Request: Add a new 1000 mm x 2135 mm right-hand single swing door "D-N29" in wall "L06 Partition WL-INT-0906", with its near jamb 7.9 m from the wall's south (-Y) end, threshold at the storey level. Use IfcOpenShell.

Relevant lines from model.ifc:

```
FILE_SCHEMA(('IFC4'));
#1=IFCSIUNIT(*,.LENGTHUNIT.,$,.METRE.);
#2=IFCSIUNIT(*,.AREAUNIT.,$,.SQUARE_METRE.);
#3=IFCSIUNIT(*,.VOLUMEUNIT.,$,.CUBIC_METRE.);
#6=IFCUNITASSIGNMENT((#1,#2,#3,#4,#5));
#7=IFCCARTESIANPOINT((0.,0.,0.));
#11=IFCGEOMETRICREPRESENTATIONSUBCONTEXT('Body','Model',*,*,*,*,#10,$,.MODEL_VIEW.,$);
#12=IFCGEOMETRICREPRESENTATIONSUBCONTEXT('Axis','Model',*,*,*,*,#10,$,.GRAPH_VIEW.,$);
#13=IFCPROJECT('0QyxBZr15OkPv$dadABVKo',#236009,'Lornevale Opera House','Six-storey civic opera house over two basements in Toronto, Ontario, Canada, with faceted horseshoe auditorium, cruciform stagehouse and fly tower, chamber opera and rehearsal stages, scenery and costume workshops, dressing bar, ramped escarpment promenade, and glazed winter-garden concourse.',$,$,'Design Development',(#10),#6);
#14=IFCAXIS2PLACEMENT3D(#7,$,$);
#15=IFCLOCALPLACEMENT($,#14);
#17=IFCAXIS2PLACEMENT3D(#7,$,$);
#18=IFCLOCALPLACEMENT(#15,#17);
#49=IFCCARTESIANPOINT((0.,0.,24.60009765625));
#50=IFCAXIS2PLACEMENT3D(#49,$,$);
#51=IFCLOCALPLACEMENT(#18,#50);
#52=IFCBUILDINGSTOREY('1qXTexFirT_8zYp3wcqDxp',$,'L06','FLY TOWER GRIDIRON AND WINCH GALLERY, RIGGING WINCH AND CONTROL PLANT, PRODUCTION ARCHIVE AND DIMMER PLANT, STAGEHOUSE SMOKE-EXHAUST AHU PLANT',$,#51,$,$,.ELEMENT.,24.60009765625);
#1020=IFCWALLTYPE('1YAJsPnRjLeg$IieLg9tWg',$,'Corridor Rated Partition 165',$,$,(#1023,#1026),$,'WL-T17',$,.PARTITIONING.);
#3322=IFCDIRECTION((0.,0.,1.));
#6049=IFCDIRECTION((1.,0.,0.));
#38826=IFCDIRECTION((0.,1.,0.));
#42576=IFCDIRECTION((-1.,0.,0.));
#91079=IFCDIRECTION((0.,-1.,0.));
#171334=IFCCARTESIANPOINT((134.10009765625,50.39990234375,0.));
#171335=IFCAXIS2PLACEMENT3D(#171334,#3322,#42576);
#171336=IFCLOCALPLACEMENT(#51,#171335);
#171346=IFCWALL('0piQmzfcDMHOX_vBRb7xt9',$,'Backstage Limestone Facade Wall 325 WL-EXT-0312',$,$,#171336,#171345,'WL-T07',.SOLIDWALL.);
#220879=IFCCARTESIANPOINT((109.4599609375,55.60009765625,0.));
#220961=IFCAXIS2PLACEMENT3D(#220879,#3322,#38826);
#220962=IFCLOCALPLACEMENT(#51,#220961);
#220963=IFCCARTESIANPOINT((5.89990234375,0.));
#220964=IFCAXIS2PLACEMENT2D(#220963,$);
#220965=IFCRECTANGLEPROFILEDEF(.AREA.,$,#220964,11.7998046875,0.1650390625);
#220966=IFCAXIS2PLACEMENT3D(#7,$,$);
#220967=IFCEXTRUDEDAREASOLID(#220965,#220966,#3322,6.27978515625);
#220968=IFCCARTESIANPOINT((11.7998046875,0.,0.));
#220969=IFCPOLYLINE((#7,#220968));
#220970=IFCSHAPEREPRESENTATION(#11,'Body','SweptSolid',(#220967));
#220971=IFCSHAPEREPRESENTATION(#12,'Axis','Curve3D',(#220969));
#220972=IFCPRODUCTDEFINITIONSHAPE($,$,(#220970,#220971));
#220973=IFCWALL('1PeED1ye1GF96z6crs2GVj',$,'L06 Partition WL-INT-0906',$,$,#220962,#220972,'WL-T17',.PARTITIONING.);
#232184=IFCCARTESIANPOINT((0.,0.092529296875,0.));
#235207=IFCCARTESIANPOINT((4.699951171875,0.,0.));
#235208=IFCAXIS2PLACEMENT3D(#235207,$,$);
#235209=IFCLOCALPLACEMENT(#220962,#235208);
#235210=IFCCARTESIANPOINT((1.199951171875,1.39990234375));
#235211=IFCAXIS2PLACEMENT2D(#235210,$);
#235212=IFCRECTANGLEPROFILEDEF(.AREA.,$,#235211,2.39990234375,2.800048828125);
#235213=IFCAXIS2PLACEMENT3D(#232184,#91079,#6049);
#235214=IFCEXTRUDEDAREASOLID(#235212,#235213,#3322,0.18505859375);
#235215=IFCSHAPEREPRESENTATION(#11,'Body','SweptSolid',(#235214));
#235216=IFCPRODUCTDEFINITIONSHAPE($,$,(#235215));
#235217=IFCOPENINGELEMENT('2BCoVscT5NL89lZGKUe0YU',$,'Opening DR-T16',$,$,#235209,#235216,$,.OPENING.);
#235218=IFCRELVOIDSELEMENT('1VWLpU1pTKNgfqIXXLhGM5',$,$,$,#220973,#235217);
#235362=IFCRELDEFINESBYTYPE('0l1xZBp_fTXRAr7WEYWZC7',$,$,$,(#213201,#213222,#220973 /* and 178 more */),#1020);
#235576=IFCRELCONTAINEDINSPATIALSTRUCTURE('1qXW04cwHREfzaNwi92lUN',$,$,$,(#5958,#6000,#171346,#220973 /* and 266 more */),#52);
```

```python
import numpy as np
import ifcopenshell
import ifcopenshell.api.feature
import ifcopenshell.api.geometry
import ifcopenshell.api.root
import ifcopenshell.api.spatial
import ifcopenshell.geom
import ifcopenshell.util.element
import ifcopenshell.util.placement
import ifcopenshell.util.representation
import ifcopenshell.util.shape
import ifcopenshell.util.unit

model = ifcopenshell.open("model.ifc")
unit_scale = ifcopenshell.util.unit.calculate_unit_scale(model)
settings = ifcopenshell.geom.settings()


def volume(element):
    """Net volume in cubic metres, openings subtracted."""
    shape = ifcopenshell.geom.create_shape(settings, element)
    return ifcopenshell.util.shape.get_volume(shape.geometry)


wall = model.by_guid("1PeED1ye1GF96z6crs2GVj")
storey = ifcopenshell.util.element.get_container(wall, ifc_class="IfcBuildingStorey")
context = ifcopenshell.util.representation.get_context(model, "Model", "Body", "MODEL_VIEW")
before = volume(wall)

width, height, from_end, sill = 1, 2.135, 7.9, 0.0  # metres

# The wall runs along its own X axis, and the end named is its -X end.
wall_shape = ifcopenshell.geom.create_shape(settings, wall)
x, y, z = ifcopenshell.util.shape.get_vertices(wall_shape.geometry).T
start = x.min() + from_end
face, thickness = float(y.min()), float(y.max() - y.min())
wall_matrix = ifcopenshell.util.placement.get_local_placement(wall.ObjectPlacement)
level = ifcopenshell.util.placement.get_local_placement(storey.ObjectPlacement)[2, 3]


def in_wall(x, y):
    """Placement at x, y metres in the wall's axes, at sill height."""
    matrix = wall_matrix.copy()
    matrix[:, 3] = wall_matrix @ np.array([x / unit_scale, y / unit_scale, 0.0, 1.0])
    matrix[2, 3] = level + sill / unit_scale
    return matrix


# Opening: a box that overshoots both wall faces by 50 mm.
opening = ifcopenshell.api.root.create_entity(model, ifc_class="IfcOpeningElement", predefined_type="OPENING")
box = ifcopenshell.api.geometry.add_wall_representation(
    model, context=context, length=width, height=height, thickness=thickness + 0.1
)
ifcopenshell.api.geometry.assign_representation(model, product=opening, representation=box)
ifcopenshell.api.geometry.edit_object_placement(model, product=opening, matrix=in_wall(start, face - 0.05), is_si=False)
ifcopenshell.api.feature.add_feature(model, feature=opening, element=wall)

door = ifcopenshell.api.root.create_entity(model, ifc_class="IfcDoor", name="D-N29", predefined_type="DOOR")
door.OverallWidth, door.OverallHeight = width / unit_scale, height / unit_scale
door.OperationType = "SINGLE_SWING_RIGHT"
body = ifcopenshell.api.geometry.add_door_representation(
    model,
    context=context,
    overall_width=door.OverallWidth,
    overall_height=door.OverallHeight,
    operation_type="SINGLE_SWING_RIGHT",
    lining_properties={"LiningDepth": thickness / unit_scale, "ThresholdDepth": thickness / unit_scale},
)
ifcopenshell.api.geometry.assign_representation(model, product=door, representation=body)
ifcopenshell.api.spatial.assign_container(model, products=[door], relating_structure=storey)
ifcopenshell.api.feature.add_filling(model, opening=opening, element=door)

# The lining spans the wall, so the door starts at the wall face.
ifcopenshell.api.geometry.edit_object_placement(model, product=door, matrix=in_wall(start, face), is_si=False)

after = volume(wall)

print(f"wall volume {before:.3f} -> {after:.3f} m3")

model.write("model_updated.ifc")
```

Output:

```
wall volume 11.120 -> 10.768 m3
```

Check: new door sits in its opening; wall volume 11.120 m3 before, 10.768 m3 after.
